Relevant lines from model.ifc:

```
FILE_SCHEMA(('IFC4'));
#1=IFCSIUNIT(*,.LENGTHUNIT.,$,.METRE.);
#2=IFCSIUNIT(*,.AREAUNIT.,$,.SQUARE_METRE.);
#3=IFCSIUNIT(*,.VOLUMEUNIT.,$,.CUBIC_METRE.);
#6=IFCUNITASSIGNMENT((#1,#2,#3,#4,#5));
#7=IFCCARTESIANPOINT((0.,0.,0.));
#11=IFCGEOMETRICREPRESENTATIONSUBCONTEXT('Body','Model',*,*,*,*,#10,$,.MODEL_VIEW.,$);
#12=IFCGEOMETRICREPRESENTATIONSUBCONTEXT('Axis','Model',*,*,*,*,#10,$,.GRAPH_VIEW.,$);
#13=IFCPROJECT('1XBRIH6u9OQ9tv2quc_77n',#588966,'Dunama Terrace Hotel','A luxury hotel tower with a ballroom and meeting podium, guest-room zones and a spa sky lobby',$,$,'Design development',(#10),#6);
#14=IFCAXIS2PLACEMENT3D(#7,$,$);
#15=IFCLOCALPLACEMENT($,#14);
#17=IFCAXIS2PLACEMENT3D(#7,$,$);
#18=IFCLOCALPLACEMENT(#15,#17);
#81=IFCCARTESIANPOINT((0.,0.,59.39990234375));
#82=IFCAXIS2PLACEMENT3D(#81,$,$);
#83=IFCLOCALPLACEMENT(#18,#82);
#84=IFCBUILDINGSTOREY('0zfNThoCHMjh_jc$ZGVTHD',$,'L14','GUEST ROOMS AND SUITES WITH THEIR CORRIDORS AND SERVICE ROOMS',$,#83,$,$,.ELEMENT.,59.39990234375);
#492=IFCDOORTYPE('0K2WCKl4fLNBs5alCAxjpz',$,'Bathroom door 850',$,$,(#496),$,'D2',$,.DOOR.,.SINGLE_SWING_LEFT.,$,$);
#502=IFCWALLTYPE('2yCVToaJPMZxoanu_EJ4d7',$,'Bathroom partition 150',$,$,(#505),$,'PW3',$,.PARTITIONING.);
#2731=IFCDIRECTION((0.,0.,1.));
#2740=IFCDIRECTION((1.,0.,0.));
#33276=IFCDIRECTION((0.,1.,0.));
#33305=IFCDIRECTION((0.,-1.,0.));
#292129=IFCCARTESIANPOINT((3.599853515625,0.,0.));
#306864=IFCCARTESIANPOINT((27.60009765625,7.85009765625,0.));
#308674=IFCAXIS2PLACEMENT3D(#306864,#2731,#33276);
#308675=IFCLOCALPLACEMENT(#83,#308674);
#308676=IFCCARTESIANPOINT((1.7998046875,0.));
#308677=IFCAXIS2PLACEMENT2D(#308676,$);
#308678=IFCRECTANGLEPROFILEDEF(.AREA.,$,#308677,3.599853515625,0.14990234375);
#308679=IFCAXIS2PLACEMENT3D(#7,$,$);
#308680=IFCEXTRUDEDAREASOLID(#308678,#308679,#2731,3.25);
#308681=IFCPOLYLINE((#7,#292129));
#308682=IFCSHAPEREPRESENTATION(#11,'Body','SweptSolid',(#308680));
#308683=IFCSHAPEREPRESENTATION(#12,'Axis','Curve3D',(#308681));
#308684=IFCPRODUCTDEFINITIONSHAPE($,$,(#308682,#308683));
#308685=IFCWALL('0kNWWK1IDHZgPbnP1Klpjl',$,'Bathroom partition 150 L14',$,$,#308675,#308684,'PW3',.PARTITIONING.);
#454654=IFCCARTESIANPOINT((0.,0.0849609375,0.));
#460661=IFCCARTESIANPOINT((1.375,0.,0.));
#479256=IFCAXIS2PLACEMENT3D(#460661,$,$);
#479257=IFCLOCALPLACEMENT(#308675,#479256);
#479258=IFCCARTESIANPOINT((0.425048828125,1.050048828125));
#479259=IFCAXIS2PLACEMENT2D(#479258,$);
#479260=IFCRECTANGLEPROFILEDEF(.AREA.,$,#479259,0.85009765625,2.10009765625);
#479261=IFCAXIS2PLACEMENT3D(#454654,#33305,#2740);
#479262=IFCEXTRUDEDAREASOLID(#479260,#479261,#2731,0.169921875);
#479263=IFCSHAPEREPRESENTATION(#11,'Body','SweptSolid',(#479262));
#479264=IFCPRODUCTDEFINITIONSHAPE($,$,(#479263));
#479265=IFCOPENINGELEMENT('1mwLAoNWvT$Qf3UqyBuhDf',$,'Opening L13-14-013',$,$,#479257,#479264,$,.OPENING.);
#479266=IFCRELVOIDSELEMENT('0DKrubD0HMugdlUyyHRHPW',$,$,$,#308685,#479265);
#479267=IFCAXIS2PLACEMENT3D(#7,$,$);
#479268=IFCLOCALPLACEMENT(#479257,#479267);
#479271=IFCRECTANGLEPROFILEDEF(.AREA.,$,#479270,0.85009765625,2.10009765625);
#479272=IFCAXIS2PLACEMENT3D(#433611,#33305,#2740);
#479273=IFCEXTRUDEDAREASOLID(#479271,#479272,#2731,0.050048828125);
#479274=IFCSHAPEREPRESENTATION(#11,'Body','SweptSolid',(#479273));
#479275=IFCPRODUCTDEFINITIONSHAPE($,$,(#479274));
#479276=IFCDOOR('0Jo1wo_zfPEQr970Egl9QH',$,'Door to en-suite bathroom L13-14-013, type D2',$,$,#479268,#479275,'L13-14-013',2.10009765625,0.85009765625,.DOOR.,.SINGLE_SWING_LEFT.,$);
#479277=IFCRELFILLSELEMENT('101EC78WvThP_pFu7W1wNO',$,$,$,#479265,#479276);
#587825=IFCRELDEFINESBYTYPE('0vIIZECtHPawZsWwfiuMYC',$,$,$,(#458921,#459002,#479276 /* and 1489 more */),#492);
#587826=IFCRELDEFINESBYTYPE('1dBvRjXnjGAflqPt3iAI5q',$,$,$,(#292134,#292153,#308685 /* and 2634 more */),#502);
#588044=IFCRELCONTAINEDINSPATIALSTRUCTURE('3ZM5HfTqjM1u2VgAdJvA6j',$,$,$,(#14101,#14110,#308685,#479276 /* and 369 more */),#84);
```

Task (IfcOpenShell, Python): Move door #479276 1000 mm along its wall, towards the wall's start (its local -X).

```python
import ifcopenshell
import ifcopenshell.api.geometry
import ifcopenshell.util.placement
import ifcopenshell.util.unit

model = ifcopenshell.open("model.ifc")
unit_scale = ifcopenshell.util.unit.calculate_unit_scale(model)

door = model.by_guid("0Jo1wo_zfPEQr970Egl9QH")
opening = door.FillsVoids[0].RelatingOpeningElement
wall = opening.VoidsElements[0].RelatingBuildingElement

wall_matrix = ifcopenshell.util.placement.get_local_placement(wall.ObjectPlacement)
shift = wall_matrix[:3, 0] * -1 / unit_scale
before = ifcopenshell.util.placement.get_local_placement(door.ObjectPlacement)[:3, 3].copy()

# The door is placed relative to its opening, so it follows when the opening moves.
matrix = ifcopenshell.util.placement.get_local_placement(opening.ObjectPlacement)
matrix[:3, 3] += shift
ifcopenshell.api.geometry.edit_object_placement(
    model, product=opening, matrix=matrix, is_si=False, should_transform_children=True
)

after = ifcopenshell.util.placement.get_local_placement(door.ObjectPlacement)[:3, 3]
print("door moved by", (after - before).round(3) + 0.0)

model.write("model_v2.ifc")
```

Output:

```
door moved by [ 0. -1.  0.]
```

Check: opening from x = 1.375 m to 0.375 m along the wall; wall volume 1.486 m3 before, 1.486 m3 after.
